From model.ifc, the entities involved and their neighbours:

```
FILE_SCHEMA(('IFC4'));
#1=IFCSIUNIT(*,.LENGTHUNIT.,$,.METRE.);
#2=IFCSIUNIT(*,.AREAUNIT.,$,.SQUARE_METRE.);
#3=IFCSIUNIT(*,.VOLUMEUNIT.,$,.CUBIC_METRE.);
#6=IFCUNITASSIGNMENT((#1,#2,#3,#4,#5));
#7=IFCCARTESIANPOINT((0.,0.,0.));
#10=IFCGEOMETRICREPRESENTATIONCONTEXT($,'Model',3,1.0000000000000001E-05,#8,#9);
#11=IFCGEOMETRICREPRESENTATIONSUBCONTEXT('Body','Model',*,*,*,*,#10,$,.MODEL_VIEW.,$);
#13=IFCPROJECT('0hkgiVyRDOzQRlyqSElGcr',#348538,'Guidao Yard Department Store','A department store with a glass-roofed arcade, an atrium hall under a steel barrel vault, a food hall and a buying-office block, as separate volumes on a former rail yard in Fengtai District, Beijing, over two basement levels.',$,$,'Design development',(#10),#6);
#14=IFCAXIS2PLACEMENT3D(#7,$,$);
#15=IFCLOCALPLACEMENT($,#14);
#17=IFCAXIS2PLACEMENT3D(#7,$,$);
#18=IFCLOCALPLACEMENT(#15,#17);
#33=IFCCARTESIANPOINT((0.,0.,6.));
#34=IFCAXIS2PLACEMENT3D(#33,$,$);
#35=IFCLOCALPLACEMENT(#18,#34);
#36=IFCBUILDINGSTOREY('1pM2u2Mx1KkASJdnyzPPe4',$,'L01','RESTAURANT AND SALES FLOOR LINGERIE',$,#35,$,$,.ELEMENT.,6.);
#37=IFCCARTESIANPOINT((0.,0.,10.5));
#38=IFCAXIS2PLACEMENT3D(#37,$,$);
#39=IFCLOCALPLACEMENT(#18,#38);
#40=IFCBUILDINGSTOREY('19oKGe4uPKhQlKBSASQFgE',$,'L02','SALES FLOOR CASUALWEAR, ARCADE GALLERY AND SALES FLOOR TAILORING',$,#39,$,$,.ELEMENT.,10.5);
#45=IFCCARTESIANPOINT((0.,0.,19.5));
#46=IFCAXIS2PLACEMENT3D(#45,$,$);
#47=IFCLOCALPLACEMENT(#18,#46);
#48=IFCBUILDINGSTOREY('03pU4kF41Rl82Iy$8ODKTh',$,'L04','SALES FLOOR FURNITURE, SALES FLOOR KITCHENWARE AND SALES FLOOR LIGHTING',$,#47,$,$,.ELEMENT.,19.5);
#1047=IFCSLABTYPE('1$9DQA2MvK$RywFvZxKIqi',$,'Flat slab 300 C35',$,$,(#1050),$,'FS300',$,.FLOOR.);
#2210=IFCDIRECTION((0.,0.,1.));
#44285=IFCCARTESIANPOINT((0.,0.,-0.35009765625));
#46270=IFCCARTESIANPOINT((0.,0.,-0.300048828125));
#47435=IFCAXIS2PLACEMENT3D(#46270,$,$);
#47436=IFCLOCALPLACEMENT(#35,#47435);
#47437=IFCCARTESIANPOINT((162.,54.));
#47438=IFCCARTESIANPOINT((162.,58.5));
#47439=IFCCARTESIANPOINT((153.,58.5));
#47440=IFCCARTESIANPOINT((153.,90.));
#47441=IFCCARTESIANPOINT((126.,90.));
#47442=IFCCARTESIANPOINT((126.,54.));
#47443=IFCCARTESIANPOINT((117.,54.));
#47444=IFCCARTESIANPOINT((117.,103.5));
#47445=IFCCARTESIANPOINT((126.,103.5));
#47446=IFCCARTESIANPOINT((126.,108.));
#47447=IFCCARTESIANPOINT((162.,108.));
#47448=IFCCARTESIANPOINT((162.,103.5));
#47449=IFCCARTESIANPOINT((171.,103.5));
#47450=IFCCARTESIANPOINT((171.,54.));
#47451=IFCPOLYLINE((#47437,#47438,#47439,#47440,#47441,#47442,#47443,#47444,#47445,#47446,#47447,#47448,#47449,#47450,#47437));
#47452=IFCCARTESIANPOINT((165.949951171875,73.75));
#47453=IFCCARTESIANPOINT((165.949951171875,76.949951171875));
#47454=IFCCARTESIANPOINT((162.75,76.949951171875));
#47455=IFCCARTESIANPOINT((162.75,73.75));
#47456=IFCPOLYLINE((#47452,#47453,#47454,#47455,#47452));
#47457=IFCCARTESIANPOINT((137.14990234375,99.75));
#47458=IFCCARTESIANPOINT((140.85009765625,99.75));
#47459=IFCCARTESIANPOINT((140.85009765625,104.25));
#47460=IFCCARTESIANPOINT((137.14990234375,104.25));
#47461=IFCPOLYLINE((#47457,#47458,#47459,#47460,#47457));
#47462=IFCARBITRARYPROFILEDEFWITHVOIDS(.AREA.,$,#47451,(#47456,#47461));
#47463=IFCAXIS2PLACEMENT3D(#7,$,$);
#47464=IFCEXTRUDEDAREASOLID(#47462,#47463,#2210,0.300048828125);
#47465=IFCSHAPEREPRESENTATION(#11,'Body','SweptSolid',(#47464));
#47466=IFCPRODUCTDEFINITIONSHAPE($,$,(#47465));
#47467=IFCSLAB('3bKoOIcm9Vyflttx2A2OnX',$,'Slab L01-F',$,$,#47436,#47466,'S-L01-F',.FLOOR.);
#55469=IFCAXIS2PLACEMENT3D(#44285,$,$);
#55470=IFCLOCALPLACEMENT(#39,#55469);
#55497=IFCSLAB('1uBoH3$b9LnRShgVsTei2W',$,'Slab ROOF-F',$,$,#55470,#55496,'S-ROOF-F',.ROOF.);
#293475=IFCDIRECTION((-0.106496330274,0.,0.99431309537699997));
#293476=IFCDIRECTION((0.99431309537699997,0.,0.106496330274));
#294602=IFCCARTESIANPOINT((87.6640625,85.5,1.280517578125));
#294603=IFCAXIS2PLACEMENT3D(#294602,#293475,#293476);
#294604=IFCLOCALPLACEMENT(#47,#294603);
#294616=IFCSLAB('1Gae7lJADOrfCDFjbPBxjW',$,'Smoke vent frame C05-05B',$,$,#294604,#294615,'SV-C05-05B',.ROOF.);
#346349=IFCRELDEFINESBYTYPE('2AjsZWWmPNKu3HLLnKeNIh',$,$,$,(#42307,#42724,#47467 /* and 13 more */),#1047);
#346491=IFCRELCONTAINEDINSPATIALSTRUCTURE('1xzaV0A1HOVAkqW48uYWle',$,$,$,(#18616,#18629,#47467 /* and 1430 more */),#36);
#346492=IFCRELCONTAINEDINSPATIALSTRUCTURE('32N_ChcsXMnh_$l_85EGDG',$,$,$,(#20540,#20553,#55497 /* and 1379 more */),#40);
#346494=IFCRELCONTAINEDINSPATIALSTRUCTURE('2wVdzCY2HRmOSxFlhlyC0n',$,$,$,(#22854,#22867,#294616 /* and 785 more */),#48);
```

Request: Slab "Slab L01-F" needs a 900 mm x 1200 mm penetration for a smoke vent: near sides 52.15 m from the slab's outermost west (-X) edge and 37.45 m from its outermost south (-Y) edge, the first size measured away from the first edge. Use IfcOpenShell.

```python
import numpy as np
import ifcopenshell
import ifcopenshell.api.feature
import ifcopenshell.api.geometry
import ifcopenshell.api.root
import ifcopenshell.geom
import ifcopenshell.util.placement
import ifcopenshell.util.representation
import ifcopenshell.util.shape
import ifcopenshell.util.unit

model = ifcopenshell.open("model.ifc")
unit_scale = ifcopenshell.util.unit.calculate_unit_scale(model)
settings = ifcopenshell.geom.settings()


def volume(element):
    """Net volume in cubic metres, openings subtracted."""
    shape = ifcopenshell.geom.create_shape(settings, element)
    return ifcopenshell.util.shape.get_volume(shape.geometry)


slab = model.by_guid("3bKoOIcm9Vyflttx2A2OnX")
before = volume(slab)

# Extent in the slab's own axes, in metres. The edges named are its -X and -Y sides.
slab_shape = ifcopenshell.geom.create_shape(settings, slab)
vertices = ifcopenshell.util.shape.get_vertices(slab_shape.geometry)
x_min, y_min, bottom = vertices.min(axis=0)
top = vertices[:, 2].max()

opening = ifcopenshell.api.root.create_entity(model, ifc_class="IfcOpeningElement", name="Smoke vent opening", predefined_type="OPENING")
context = ifcopenshell.util.representation.get_context(model, "Model", "Body", "MODEL_VIEW")
width, depth = 0.9, 1.2
outline = [(0.0, 0.0), (width, 0.0), (width, depth), (0.0, depth), (0.0, 0.0)]
# Overshoot both faces by 50 mm so the cut is clean.
shape = ifcopenshell.api.geometry.add_slab_representation(
    model, context=context, depth=top - bottom + 0.1, polyline=outline
)
ifcopenshell.api.geometry.assign_representation(model, product=opening, representation=shape)

matrix = ifcopenshell.util.placement.get_local_placement(slab.ObjectPlacement)
matrix[:, 3] = matrix @ np.append(np.array([x_min + 52.15, y_min + 37.45, bottom - 0.05]) / unit_scale, 1.0)
ifcopenshell.api.geometry.edit_object_placement(model, product=opening, matrix=matrix, is_si=False)
ifcopenshell.api.feature.add_feature(model, feature=opening, element=slab)

after = volume(slab)

print(f"slab volume {before:.3f} -> {after:.3f} m3")

model.write("model_rev.ifc")
```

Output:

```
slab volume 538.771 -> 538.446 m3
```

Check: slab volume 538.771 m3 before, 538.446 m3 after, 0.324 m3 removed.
